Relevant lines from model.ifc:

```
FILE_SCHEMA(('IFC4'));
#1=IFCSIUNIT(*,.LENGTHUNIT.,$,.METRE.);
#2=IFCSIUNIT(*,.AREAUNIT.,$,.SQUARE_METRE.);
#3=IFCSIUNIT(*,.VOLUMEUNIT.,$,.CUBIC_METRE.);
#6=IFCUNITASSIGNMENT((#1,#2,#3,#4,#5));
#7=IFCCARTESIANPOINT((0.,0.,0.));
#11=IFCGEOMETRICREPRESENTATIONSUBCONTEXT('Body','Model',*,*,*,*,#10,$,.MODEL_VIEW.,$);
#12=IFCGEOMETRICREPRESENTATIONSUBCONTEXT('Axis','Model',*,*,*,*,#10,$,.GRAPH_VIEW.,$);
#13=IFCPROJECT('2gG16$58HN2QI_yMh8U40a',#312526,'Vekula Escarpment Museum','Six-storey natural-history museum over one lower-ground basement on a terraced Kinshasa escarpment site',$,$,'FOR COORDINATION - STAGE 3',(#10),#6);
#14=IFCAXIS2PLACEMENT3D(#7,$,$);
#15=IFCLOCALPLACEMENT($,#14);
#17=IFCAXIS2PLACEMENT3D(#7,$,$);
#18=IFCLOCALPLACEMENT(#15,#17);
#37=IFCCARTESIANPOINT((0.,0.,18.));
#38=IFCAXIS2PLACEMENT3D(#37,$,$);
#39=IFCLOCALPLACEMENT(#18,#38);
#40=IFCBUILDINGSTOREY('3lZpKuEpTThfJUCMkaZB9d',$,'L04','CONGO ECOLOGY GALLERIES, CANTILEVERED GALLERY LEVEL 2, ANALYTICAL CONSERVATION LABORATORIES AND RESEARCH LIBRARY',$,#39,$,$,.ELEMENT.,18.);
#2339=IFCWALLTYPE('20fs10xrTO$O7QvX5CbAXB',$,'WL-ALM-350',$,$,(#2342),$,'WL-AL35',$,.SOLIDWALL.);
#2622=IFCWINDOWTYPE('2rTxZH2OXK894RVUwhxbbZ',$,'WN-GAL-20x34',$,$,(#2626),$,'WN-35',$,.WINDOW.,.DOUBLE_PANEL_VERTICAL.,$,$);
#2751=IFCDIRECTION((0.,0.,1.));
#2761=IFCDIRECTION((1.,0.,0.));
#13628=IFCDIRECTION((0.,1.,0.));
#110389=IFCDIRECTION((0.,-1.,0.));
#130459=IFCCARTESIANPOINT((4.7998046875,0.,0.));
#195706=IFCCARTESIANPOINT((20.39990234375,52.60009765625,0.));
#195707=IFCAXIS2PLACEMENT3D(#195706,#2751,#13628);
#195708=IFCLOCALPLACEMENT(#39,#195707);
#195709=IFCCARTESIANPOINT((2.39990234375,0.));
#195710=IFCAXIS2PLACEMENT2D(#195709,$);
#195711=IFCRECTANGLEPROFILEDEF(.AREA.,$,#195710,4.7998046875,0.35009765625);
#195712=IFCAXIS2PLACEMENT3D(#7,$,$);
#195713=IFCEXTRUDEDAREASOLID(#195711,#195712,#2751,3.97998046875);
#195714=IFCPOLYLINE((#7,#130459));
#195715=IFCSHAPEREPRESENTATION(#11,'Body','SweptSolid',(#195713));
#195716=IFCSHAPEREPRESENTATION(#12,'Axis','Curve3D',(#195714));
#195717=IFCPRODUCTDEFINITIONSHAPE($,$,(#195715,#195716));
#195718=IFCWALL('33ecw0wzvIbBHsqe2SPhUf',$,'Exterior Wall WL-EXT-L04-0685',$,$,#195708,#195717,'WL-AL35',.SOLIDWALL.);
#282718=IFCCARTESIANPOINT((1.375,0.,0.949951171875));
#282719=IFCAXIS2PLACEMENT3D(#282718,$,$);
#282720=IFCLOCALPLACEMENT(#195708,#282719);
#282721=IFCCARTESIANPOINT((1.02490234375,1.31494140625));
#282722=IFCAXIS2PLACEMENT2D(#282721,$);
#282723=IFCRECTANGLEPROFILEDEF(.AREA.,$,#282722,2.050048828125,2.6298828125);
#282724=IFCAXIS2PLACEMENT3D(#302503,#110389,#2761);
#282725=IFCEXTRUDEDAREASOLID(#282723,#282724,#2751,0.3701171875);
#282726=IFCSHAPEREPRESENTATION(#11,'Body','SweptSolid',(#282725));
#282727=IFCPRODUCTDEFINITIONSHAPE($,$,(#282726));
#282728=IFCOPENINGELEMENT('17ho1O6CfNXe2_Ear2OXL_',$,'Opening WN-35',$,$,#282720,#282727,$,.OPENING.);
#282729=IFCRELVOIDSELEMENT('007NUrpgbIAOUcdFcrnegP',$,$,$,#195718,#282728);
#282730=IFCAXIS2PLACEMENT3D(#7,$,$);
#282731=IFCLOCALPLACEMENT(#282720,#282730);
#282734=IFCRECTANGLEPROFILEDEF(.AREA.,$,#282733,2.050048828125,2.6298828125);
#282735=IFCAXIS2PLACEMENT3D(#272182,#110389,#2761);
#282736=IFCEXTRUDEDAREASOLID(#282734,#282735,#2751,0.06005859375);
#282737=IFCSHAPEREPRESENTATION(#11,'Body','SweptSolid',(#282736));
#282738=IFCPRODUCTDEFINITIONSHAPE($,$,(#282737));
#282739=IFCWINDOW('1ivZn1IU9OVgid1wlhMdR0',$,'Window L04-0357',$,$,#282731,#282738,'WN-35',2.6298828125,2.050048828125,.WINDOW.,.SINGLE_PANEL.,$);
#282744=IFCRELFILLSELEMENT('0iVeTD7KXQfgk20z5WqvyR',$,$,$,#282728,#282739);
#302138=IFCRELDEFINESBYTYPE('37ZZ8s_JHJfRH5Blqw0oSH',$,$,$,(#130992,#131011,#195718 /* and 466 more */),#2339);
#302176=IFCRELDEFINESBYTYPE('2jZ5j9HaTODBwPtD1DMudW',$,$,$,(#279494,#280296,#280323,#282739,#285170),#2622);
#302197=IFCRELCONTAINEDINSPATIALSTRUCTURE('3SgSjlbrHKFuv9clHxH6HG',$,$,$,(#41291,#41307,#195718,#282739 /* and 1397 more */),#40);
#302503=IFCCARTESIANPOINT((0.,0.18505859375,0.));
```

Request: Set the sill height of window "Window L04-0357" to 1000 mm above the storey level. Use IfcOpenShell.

```python
import numpy as np
import ifcopenshell
import ifcopenshell.api.geometry
import ifcopenshell.geom
import ifcopenshell.util.element
import ifcopenshell.util.placement
import ifcopenshell.util.shape
import ifcopenshell.util.unit

model = ifcopenshell.open("model.ifc")
unit_scale = ifcopenshell.util.unit.calculate_unit_scale(model)

window = model.by_guid("1ivZn1IU9OVgid1wlhMdR0")
opening = window.FillsVoids[0].RelatingOpeningElement
storey = ifcopenshell.util.element.get_container(window, ifc_class="IfcBuildingStorey")
level = ifcopenshell.util.placement.get_local_placement(storey.ObjectPlacement)[2, 3]

# The opening's origin need not be at the sill, so measure its lowest point.
shape = ifcopenshell.geom.create_shape(ifcopenshell.geom.settings(), opening)
bottom = ifcopenshell.util.shape.get_shape_bottom_elevation(shape, shape.geometry) / unit_scale
dz = level + 1.0 - bottom

shift = np.array([0.0, 0.0, dz])
# The window is placed relative to its opening, so it follows when the opening moves.
matrix = ifcopenshell.util.placement.get_local_placement(opening.ObjectPlacement)
matrix[:3, 3] += shift
ifcopenshell.api.geometry.edit_object_placement(
    model, product=opening, matrix=matrix, is_si=False, should_transform_children=True
)

print(f"moved by {dz * unit_scale:+.3f} m")

model.write("model_edited.ifc")
```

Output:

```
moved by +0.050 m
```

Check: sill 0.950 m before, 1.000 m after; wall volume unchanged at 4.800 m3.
